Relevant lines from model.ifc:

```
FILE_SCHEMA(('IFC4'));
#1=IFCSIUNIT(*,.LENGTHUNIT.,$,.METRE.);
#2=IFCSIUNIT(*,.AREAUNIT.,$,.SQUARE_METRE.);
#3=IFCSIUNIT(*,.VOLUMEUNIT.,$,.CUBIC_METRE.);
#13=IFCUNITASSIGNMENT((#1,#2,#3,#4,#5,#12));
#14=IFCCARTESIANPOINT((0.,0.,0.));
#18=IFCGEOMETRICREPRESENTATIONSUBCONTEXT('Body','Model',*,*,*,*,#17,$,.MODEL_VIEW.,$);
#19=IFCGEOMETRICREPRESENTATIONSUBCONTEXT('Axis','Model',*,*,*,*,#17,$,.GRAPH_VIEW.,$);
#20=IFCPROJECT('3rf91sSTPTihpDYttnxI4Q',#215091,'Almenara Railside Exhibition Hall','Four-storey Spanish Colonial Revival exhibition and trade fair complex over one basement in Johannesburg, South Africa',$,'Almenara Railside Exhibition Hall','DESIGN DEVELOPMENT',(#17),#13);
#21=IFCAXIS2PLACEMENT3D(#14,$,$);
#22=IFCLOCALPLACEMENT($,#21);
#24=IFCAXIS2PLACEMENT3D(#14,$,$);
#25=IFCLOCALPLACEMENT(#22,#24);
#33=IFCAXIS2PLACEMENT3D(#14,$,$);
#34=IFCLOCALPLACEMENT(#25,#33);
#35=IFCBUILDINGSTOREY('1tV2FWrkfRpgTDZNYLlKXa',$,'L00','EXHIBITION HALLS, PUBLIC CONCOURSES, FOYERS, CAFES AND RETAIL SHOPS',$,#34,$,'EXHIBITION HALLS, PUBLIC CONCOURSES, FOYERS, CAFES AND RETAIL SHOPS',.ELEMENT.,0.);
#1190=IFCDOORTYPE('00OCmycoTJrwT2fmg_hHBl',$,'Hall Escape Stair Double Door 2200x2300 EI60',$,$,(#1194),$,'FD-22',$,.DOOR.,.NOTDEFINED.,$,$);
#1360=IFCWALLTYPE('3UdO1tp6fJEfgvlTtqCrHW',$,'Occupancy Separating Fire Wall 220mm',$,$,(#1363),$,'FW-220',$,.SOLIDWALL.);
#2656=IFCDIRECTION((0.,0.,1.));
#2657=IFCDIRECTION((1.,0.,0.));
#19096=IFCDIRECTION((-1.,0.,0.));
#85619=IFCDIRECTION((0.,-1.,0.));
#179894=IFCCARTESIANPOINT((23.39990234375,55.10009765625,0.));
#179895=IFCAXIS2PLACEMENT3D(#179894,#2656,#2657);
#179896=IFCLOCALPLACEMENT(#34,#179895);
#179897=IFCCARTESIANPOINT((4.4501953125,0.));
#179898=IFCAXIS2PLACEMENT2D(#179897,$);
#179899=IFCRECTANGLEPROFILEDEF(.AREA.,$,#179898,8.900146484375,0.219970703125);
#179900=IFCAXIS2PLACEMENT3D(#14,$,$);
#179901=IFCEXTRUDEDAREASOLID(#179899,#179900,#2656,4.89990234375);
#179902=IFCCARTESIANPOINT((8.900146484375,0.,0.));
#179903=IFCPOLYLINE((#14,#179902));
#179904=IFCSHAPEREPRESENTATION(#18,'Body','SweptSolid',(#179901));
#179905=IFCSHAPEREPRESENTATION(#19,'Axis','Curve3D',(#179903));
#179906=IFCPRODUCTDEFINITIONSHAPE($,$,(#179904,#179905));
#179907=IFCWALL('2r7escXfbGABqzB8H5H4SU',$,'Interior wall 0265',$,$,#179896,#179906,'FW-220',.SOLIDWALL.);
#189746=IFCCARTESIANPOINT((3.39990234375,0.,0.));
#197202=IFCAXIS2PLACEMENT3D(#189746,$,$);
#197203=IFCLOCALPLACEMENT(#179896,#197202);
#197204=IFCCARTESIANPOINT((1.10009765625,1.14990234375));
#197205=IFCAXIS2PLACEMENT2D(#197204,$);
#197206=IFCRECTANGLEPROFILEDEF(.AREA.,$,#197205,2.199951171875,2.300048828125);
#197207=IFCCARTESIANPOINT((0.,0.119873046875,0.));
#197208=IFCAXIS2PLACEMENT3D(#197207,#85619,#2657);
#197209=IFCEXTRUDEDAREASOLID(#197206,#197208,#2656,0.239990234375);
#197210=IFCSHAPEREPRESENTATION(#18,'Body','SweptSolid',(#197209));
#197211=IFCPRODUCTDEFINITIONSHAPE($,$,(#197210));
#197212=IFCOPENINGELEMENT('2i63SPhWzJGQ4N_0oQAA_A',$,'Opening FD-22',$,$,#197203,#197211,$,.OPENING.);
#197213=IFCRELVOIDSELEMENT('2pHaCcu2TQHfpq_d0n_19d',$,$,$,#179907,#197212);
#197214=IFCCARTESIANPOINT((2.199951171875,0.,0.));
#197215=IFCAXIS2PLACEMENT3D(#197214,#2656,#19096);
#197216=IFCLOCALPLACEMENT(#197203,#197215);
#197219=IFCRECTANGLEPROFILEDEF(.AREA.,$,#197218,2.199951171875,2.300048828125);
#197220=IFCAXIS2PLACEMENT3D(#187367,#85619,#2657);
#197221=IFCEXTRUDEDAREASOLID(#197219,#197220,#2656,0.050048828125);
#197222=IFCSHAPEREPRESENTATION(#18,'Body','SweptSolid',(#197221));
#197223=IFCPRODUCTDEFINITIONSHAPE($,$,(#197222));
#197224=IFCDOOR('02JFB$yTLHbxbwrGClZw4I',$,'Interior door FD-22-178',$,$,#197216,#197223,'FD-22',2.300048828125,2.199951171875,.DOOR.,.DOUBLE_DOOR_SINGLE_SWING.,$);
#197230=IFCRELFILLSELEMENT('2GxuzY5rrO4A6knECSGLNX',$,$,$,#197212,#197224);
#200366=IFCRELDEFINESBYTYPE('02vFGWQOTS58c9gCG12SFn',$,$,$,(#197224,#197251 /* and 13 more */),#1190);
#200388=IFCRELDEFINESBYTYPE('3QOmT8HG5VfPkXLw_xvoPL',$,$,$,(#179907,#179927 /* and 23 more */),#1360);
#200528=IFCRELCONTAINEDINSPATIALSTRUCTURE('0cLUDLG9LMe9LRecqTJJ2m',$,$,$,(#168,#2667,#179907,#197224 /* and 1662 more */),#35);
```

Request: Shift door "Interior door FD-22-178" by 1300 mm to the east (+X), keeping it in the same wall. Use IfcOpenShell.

```python
import ifcopenshell
import ifcopenshell.api.geometry
import ifcopenshell.util.placement
import ifcopenshell.util.unit

model = ifcopenshell.open("model.ifc")
unit_scale = ifcopenshell.util.unit.calculate_unit_scale(model)

door = model.by_guid("02JFB$yTLHbxbwrGClZw4I")
opening = door.FillsVoids[0].RelatingOpeningElement
wall = opening.VoidsElements[0].RelatingBuildingElement

wall_matrix = ifcopenshell.util.placement.get_local_placement(wall.ObjectPlacement)
shift = wall_matrix[:3, 0] * 1.3 / unit_scale
before = ifcopenshell.util.placement.get_local_placement(door.ObjectPlacement)[:3, 3].copy()

# The door is placed relative to its opening, so it follows when the opening moves.
matrix = ifcopenshell.util.placement.get_local_placement(opening.ObjectPlacement)
matrix[:3, 3] += shift
ifcopenshell.api.geometry.edit_object_placement(
    model, product=opening, matrix=matrix, is_si=False, should_transform_children=True
)

after = ifcopenshell.util.placement.get_local_placement(door.ObjectPlacement)[:3, 3]
print("door moved by", (after - before).round(3) + 0.0)

model.write("model_v2.ifc")
```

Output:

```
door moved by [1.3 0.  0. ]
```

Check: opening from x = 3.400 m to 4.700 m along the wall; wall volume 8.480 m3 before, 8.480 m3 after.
